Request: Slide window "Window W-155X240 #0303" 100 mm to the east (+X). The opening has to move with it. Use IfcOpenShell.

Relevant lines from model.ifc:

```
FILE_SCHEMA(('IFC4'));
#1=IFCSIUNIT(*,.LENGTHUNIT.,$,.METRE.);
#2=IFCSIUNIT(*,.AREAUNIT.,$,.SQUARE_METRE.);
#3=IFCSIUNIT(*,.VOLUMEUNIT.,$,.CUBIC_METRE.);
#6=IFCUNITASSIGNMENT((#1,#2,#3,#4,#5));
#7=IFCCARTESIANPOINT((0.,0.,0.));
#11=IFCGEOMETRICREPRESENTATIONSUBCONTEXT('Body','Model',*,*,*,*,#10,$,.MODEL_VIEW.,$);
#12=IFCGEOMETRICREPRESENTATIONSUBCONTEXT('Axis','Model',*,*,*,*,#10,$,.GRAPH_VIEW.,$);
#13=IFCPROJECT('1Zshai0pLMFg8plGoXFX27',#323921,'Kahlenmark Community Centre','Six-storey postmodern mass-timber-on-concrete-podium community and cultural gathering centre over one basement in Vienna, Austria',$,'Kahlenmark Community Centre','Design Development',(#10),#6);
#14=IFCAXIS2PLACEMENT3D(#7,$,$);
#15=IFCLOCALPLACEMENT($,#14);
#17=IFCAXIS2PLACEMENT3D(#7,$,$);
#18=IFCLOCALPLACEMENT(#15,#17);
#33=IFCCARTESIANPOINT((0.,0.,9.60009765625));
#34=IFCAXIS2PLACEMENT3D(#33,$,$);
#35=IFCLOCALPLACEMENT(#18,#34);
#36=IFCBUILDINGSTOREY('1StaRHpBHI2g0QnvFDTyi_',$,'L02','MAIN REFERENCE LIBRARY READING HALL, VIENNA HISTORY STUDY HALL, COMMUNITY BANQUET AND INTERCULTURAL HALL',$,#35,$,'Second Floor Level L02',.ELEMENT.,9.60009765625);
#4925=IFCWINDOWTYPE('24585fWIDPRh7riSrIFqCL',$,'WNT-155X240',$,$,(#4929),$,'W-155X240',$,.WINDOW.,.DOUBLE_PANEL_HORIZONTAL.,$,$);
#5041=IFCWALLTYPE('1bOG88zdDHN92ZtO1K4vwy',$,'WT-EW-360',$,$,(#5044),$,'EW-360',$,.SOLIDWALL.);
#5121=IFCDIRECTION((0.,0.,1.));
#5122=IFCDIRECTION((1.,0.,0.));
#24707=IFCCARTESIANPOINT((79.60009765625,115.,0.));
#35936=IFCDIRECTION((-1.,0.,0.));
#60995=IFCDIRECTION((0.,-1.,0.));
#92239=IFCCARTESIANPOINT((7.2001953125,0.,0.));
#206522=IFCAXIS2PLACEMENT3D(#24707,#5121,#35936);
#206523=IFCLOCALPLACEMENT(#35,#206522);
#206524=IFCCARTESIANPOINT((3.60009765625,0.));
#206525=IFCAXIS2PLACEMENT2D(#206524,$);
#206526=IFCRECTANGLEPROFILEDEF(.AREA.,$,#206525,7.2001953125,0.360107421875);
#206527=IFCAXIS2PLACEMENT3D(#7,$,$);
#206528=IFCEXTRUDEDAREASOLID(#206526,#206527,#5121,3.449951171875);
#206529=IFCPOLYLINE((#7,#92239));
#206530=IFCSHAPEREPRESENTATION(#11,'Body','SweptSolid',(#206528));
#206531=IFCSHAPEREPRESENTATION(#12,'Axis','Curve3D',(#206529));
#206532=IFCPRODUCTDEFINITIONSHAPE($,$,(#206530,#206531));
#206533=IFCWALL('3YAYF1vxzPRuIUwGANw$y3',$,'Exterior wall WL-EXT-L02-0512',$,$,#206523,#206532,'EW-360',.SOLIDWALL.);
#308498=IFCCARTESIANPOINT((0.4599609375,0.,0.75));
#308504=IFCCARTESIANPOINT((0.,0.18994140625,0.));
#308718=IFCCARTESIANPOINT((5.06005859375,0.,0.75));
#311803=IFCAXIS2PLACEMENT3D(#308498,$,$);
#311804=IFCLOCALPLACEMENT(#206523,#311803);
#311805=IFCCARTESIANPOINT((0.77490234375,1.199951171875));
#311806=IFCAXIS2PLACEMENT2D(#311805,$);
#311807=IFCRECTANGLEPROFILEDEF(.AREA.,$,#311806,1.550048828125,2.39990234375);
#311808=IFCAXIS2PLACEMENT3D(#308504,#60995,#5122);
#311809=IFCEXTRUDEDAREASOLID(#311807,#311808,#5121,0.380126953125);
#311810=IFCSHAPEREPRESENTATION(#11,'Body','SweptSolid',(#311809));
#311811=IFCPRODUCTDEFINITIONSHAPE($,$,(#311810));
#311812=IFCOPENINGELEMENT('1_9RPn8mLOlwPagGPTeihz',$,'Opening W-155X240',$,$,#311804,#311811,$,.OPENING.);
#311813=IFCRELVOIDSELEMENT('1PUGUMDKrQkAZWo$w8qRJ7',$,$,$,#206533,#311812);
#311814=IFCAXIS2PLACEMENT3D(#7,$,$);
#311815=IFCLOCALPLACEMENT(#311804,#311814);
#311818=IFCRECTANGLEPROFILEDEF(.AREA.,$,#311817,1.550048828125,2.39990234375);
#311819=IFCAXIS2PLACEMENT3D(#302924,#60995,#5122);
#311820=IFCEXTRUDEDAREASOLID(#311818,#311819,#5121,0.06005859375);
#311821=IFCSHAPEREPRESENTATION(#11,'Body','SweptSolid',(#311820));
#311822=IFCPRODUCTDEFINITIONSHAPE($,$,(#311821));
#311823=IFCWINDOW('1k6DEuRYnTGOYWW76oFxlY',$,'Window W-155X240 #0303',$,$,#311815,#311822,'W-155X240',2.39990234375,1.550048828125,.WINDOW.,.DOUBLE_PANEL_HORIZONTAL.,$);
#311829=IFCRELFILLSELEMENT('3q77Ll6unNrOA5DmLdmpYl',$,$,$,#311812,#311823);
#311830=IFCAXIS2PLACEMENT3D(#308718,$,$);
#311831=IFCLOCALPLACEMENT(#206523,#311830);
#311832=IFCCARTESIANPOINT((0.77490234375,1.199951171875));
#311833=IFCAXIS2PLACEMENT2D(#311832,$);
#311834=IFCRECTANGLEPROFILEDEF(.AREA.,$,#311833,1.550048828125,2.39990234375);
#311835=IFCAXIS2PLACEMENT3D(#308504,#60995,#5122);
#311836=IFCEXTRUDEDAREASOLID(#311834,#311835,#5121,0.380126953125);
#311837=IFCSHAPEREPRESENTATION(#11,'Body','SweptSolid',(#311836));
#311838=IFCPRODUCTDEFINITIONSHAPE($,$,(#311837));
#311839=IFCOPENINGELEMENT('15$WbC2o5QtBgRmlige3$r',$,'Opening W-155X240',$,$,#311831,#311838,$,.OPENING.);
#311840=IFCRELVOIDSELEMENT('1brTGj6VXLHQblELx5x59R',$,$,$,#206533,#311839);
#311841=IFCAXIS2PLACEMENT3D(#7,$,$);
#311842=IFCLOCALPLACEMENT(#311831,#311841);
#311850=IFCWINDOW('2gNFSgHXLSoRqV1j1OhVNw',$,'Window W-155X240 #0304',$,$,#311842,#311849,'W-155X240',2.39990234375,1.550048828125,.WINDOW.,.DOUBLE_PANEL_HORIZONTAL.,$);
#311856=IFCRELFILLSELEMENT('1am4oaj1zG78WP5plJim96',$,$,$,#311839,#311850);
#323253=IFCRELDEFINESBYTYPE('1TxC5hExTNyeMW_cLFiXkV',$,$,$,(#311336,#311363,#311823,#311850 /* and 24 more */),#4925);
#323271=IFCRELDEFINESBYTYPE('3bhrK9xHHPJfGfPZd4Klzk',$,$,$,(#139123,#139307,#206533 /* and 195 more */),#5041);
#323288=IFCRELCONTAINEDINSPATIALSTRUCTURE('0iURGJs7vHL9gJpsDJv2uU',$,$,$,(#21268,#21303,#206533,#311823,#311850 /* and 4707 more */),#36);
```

```python
import ifcopenshell
import ifcopenshell.api.geometry
import ifcopenshell.util.placement

model = ifcopenshell.open("model.ifc")

window = model.by_id(311823)
opening = window.FillsVoids[0].RelatingOpeningElement
wall = opening.VoidsElements[0].RelatingBuildingElement

wall_matrix = ifcopenshell.util.placement.get_local_placement(wall.ObjectPlacement)
shift = wall_matrix[:3, 0] * -0.1
before = ifcopenshell.util.placement.get_local_placement(window.ObjectPlacement)[:3, 3].copy()

# The window is placed relative to its opening, so it follows when the opening moves.
matrix = ifcopenshell.util.placement.get_local_placement(opening.ObjectPlacement)
matrix[:3, 3] += shift
ifcopenshell.api.geometry.edit_object_placement(
    model, product=opening, matrix=matrix, is_si=False, should_transform_children=True
)

after = ifcopenshell.util.placement.get_local_placement(window.ObjectPlacement)[:3, 3]
print("window moved by", (after - before).round(3) + 0.0)

model.write("model_v2.ifc")
```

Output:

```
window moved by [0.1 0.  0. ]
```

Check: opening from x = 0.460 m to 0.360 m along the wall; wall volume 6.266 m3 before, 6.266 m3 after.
